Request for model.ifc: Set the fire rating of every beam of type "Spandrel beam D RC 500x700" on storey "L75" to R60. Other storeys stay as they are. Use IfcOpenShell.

First a look at what the model holds.

```python
import ifcopenshell
import ifcopenshell.util.element

model = ifcopenshell.open("model.ifc")
print(model.schema)
storey = next(s for s in model.by_type("IfcBuildingStorey") if s.Name == "L75")
beams = [e for e in ifcopenshell.util.element.get_decomposition(storey) if e.is_a("IfcBeam")]
seen = {}
for e in beams:
    element_type = ifcopenshell.util.element.get_type(e)
    key = (element_type.Name if element_type != e and element_type else None, ifcopenshell.util.element.get_pset(e, "Pset_BeamCommon", "FireRating"))
    seen[key] = seen.get(key, 0) + 1
for (name, value), count in sorted(seen.items(), key=str):
    print(count, "x", name, "|", value)
```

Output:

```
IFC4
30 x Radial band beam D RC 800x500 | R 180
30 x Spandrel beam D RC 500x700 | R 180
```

```python
import ifcopenshell
import ifcopenshell.api.pset
import ifcopenshell.util.element

model = ifcopenshell.open("model.ifc")

storey = next(s for s in model.by_type("IfcBuildingStorey") if s.Name == "L75")
beams = [e for e in ifcopenshell.util.element.get_decomposition(storey) if e.is_a("IfcBeam")]

count = 0
for e in beams:
    element_type = ifcopenshell.util.element.get_type(e)
    if element_type in (None, e) or element_type.Name != "Spandrel beam D RC 500x700":
        continue
    found = ifcopenshell.util.element.get_pset(e, "Pset_BeamCommon", should_inherit=False)
    if found:
        pset = model.by_id(found["id"])
        if len(ifcopenshell.util.element.get_elements_by_pset(pset)) > 1:
            pset = ifcopenshell.api.pset.unshare_pset(model, products=[e], pset=pset)[0]
    else:
        pset = ifcopenshell.api.pset.add_pset(model, product=e, name="Pset_BeamCommon")
    ifcopenshell.api.pset.edit_pset(model, pset=pset, properties={"FireRating": "R60"})
    count += 1

print(count, "beams updated")

model.write("model_updated.ifc")
```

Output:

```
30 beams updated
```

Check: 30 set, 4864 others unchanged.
